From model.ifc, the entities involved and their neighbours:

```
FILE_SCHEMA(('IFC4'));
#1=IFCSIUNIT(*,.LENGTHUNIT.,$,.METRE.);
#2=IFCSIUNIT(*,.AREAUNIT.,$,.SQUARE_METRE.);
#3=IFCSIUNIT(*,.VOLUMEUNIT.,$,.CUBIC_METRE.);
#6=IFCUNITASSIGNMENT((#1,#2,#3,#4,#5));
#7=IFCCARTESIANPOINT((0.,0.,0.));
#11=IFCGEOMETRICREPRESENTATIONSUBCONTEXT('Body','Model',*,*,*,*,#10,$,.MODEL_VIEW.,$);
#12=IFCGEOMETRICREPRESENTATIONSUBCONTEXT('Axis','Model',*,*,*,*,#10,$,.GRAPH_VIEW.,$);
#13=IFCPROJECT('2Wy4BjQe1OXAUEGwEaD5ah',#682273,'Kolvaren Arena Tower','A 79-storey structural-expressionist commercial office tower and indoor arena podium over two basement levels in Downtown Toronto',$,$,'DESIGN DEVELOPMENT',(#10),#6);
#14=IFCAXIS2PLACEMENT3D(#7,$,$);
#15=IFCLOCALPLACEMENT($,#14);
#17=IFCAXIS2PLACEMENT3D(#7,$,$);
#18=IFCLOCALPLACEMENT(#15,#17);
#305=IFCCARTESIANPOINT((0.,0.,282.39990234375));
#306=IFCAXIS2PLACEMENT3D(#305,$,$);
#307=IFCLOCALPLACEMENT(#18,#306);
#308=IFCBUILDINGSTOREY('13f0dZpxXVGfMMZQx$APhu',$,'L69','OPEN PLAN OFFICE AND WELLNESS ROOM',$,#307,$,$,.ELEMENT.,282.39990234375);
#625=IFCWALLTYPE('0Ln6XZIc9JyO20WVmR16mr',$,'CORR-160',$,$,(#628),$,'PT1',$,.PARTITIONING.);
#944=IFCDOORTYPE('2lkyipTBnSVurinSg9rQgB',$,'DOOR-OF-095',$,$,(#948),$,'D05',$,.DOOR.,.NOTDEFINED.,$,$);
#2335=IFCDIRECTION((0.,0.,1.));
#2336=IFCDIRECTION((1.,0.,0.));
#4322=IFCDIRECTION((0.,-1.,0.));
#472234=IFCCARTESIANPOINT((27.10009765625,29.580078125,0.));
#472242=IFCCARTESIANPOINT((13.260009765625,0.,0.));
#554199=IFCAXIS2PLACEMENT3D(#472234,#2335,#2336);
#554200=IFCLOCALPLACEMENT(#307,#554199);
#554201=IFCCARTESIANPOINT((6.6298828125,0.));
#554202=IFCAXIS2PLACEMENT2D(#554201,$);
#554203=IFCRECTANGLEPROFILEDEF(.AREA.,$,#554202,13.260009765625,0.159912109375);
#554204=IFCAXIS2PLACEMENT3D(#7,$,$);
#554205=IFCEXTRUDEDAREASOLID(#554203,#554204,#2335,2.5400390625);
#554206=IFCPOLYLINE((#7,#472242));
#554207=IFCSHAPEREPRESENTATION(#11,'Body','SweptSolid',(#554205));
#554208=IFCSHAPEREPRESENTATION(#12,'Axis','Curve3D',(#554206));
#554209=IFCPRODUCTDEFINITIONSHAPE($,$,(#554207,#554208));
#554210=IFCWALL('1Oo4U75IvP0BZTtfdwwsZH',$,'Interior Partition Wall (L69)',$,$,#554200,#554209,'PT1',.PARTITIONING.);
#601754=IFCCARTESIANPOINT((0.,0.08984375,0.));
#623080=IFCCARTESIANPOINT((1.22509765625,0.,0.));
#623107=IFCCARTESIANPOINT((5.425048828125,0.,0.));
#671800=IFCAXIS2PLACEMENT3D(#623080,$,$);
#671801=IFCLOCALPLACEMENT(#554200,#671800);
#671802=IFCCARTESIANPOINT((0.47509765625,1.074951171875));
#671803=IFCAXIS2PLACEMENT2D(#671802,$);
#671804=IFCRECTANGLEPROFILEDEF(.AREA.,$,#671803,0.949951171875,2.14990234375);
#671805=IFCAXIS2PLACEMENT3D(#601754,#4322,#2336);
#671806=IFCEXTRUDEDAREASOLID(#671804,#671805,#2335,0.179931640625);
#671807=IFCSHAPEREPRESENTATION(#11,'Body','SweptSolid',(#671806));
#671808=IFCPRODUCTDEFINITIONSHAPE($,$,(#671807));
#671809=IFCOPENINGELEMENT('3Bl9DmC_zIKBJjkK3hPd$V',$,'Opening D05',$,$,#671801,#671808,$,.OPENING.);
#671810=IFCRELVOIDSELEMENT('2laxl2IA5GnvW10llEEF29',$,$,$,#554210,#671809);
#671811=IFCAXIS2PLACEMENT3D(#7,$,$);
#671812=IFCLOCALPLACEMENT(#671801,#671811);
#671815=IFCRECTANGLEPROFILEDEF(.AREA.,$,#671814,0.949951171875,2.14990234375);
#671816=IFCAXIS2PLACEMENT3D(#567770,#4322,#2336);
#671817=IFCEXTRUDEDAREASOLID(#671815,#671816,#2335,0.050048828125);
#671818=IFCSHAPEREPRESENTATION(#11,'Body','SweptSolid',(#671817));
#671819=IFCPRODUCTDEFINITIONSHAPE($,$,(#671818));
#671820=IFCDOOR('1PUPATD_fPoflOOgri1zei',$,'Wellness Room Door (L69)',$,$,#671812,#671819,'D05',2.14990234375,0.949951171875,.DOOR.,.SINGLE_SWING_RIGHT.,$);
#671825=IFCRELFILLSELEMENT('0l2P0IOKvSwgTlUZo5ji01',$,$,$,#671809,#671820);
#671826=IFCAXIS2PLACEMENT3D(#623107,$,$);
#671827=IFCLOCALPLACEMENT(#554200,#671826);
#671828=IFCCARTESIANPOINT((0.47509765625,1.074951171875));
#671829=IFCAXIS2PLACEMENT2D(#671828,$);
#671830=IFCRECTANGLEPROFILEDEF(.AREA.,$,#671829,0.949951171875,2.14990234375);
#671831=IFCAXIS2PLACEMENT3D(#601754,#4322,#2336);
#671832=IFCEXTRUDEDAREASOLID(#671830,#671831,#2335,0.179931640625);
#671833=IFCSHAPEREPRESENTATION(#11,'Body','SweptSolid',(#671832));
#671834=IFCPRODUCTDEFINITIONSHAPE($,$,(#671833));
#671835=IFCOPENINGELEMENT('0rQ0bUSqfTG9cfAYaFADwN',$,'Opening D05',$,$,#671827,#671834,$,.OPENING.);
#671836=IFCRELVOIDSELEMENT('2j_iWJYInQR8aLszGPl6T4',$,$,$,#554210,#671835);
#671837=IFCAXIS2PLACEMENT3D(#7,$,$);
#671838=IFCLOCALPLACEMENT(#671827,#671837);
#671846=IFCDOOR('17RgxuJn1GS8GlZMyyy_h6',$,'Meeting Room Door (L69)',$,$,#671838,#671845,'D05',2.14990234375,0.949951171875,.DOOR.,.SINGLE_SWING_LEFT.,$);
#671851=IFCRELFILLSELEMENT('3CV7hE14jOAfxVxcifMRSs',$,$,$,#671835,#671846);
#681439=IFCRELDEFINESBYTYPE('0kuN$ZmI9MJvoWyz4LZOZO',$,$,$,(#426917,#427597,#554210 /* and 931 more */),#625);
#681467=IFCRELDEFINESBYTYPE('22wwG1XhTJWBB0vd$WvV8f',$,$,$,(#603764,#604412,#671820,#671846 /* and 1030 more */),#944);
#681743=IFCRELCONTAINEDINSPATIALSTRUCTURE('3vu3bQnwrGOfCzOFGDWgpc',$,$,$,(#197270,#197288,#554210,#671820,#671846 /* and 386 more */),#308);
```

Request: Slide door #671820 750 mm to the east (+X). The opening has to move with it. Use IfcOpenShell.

```python
import ifcopenshell
import ifcopenshell.api.geometry
import ifcopenshell.util.placement
import ifcopenshell.util.unit

model = ifcopenshell.open("model.ifc")
unit_scale = ifcopenshell.util.unit.calculate_unit_scale(model)

door = model.by_guid("1PUPATD_fPoflOOgri1zei")
opening = door.FillsVoids[0].RelatingOpeningElement
wall = opening.VoidsElements[0].RelatingBuildingElement

wall_matrix = ifcopenshell.util.placement.get_local_placement(wall.ObjectPlacement)
shift = wall_matrix[:3, 0] * 0.75 / unit_scale
before = ifcopenshell.util.placement.get_local_placement(door.ObjectPlacement)[:3, 3].copy()

# The door is placed relative to its opening, so it follows when the opening moves.
matrix = ifcopenshell.util.placement.get_local_placement(opening.ObjectPlacement)
matrix[:3, 3] += shift
ifcopenshell.api.geometry.edit_object_placement(
    model, product=opening, matrix=matrix, is_si=False, should_transform_children=True
)

after = ifcopenshell.util.placement.get_local_placement(door.ObjectPlacement)[:3, 3]
print("door moved by", (after - before).round(3) + 0.0)

model.write("model_rev.ifc")
```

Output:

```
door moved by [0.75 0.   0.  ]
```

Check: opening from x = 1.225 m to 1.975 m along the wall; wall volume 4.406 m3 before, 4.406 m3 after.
